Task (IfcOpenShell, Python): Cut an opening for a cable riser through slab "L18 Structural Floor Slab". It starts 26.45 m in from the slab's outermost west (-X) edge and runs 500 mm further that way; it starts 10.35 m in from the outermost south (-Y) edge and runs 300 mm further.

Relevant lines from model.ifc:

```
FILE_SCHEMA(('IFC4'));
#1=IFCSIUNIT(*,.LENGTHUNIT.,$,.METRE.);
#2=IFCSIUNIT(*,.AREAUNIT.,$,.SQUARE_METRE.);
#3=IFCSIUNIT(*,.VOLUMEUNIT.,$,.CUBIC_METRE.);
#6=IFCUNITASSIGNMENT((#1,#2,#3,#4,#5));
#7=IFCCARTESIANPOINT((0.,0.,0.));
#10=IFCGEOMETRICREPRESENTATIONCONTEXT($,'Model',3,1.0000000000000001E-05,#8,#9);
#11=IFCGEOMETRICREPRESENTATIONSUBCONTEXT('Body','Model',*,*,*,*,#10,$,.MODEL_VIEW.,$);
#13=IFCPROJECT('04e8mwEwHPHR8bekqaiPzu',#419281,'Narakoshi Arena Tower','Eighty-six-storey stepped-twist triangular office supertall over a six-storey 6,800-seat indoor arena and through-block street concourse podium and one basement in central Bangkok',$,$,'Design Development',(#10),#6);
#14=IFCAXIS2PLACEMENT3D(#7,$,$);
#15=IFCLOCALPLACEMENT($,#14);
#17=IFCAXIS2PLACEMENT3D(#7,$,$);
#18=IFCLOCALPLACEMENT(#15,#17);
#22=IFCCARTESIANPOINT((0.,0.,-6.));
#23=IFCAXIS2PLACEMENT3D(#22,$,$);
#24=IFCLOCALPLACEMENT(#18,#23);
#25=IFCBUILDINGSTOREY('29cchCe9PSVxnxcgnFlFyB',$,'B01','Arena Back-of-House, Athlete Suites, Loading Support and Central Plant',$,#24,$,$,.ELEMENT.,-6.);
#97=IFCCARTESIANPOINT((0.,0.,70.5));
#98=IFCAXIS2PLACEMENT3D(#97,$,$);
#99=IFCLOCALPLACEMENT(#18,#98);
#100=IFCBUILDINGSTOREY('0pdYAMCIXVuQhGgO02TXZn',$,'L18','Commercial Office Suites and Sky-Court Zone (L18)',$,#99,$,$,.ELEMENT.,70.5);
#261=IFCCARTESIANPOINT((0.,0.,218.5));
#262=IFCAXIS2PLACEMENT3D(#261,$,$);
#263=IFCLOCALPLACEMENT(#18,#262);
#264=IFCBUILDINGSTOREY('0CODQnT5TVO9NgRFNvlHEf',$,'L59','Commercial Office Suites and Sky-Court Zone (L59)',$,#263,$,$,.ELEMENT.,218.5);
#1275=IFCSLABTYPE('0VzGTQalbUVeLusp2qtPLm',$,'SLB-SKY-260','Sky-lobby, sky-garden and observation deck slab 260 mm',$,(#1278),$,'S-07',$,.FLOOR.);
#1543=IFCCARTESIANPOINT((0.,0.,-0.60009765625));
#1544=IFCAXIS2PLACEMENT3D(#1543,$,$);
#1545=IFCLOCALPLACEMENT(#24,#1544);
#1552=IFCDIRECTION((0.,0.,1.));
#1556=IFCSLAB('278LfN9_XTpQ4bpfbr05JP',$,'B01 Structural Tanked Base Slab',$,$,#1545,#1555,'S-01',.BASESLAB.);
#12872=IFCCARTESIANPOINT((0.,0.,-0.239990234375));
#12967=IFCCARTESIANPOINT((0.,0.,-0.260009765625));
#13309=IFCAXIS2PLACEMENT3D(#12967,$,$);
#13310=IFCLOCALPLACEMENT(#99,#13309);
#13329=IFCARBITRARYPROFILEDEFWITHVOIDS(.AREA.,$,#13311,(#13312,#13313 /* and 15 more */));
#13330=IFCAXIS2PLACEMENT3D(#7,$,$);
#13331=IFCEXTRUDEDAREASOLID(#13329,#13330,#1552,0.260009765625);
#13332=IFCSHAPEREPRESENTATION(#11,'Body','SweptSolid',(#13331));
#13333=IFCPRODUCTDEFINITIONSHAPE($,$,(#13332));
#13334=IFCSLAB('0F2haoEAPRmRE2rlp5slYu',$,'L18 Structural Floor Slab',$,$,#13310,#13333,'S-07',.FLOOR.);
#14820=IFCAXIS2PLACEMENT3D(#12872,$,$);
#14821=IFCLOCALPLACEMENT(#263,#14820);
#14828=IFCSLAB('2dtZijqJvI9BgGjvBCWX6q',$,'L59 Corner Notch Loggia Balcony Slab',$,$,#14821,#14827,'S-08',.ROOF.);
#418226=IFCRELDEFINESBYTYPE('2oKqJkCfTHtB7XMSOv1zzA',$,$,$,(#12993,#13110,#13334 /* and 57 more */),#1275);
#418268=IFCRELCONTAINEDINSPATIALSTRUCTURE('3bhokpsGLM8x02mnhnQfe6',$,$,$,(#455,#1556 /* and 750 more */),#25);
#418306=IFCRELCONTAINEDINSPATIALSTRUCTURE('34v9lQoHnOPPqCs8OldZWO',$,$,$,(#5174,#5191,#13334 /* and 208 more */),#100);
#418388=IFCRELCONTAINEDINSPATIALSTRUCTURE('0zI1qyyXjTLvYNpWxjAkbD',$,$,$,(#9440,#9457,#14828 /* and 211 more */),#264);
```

```python
import numpy as np
import ifcopenshell
import ifcopenshell.api.feature
import ifcopenshell.api.geometry
import ifcopenshell.api.root
import ifcopenshell.geom
import ifcopenshell.util.placement
import ifcopenshell.util.representation
import ifcopenshell.util.shape
import ifcopenshell.util.unit

model = ifcopenshell.open("model.ifc")
unit_scale = ifcopenshell.util.unit.calculate_unit_scale(model)
settings = ifcopenshell.geom.settings()


def volume(element):
    """Net volume in cubic metres, openings subtracted."""
    shape = ifcopenshell.geom.create_shape(settings, element)
    return ifcopenshell.util.shape.get_volume(shape.geometry)


slab = model.by_guid("0F2haoEAPRmRE2rlp5slYu")
before = volume(slab)

# Extent in the slab's own axes, in metres. The edges named are its -X and -Y sides.
slab_shape = ifcopenshell.geom.create_shape(settings, slab)
vertices = ifcopenshell.util.shape.get_vertices(slab_shape.geometry)
x_min, y_min, bottom = vertices.min(axis=0)
top = vertices[:, 2].max()

opening = ifcopenshell.api.root.create_entity(model, ifc_class="IfcOpeningElement", name="Cable riser opening", predefined_type="OPENING")
context = ifcopenshell.util.representation.get_context(model, "Model", "Body", "MODEL_VIEW")
width, depth = 0.5, 0.3
outline = [(0.0, 0.0), (width, 0.0), (width, depth), (0.0, depth), (0.0, 0.0)]
# Overshoot both faces by 50 mm so the cut is clean.
shape = ifcopenshell.api.geometry.add_slab_representation(
    model, context=context, depth=top - bottom + 0.1, polyline=outline
)
ifcopenshell.api.geometry.assign_representation(model, product=opening, representation=shape)

matrix = ifcopenshell.util.placement.get_local_placement(slab.ObjectPlacement)
matrix[:, 3] = matrix @ np.append(np.array([x_min + 26.45, y_min + 10.35, bottom - 0.05]) / unit_scale, 1.0)
ifcopenshell.api.geometry.edit_object_placement(model, product=opening, matrix=matrix, is_si=False)
ifcopenshell.api.feature.add_feature(model, feature=opening, element=slab)

after = volume(slab)

print(f"slab volume {before:.3f} -> {after:.3f} m3")

model.write("model-out.ifc")
```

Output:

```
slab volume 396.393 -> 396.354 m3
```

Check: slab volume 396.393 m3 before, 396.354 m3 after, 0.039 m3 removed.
